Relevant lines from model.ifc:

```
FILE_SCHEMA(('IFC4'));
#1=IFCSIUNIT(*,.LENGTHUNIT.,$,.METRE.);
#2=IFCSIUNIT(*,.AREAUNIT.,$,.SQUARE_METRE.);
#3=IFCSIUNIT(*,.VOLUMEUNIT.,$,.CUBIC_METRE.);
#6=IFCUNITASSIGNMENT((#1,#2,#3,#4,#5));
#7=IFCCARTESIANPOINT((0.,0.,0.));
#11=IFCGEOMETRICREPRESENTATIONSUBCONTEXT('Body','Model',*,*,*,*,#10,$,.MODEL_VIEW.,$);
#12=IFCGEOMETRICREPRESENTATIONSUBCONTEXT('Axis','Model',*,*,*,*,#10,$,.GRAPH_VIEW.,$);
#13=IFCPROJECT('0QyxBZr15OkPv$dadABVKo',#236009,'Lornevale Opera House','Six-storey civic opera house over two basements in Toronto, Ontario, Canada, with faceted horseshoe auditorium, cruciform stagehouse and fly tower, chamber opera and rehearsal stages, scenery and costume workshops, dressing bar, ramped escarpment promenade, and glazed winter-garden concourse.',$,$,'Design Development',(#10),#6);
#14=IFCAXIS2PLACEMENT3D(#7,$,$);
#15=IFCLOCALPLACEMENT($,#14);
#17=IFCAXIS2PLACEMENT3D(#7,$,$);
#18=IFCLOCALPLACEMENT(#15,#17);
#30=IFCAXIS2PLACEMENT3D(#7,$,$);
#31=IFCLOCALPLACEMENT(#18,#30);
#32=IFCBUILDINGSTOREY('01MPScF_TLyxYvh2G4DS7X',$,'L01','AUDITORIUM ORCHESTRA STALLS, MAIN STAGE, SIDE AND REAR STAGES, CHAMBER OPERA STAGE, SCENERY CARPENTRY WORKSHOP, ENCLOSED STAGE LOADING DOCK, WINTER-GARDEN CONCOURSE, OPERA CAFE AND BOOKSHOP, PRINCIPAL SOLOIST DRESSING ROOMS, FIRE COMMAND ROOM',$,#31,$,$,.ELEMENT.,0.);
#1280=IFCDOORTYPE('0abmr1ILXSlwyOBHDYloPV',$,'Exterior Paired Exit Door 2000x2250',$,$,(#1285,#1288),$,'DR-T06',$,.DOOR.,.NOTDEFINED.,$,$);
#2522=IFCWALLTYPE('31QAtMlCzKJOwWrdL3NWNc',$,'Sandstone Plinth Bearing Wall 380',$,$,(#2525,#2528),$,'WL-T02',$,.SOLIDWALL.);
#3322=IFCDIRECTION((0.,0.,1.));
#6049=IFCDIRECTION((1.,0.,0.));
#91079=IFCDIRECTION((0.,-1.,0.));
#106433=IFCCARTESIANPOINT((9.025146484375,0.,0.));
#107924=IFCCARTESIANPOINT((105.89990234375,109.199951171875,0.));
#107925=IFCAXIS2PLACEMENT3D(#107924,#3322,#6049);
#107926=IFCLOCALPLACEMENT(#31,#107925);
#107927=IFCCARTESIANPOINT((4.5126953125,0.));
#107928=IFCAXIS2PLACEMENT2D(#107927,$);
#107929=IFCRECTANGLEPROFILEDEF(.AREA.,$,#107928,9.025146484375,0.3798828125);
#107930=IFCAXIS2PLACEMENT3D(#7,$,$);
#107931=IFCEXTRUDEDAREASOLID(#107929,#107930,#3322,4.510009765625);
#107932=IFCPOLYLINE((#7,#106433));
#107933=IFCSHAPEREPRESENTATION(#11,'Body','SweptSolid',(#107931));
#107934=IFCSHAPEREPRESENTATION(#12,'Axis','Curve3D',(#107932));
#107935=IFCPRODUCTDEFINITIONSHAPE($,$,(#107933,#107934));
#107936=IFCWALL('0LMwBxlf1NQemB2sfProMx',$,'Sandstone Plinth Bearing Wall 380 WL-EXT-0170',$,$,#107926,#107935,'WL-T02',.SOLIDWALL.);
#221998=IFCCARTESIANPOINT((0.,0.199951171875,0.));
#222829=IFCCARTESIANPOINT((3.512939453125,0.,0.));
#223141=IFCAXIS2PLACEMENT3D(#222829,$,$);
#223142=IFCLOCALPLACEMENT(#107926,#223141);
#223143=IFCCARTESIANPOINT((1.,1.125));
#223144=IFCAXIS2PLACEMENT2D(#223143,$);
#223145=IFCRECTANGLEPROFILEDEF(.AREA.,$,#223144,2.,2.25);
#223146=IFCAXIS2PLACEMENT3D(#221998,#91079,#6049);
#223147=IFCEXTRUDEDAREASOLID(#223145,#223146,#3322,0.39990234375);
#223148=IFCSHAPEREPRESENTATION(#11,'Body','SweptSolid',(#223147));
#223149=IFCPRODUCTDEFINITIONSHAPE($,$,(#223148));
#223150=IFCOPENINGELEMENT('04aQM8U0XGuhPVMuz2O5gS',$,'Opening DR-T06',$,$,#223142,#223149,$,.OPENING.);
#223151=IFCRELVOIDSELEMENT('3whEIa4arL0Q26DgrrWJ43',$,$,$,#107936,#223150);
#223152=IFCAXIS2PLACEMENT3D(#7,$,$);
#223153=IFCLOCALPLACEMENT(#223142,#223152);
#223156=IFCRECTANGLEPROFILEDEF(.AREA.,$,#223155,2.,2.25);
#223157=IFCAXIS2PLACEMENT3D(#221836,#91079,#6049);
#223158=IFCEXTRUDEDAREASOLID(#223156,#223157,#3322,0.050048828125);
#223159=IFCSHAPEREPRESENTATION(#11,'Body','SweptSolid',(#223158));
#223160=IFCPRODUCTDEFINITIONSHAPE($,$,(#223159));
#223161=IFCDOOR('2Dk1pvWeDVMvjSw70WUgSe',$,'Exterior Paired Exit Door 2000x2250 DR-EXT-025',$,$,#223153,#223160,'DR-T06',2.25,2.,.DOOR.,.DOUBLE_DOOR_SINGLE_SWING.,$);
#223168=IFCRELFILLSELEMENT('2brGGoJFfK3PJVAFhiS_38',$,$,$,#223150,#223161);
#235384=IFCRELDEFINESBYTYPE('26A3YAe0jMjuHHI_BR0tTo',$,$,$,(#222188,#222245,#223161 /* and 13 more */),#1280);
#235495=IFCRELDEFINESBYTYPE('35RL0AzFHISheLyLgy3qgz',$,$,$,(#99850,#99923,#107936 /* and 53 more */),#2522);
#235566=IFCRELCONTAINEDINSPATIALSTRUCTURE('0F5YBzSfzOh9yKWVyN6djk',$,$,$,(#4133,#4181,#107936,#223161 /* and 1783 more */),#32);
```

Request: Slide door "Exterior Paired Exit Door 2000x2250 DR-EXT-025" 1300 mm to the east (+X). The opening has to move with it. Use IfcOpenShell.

```python
import ifcopenshell
import ifcopenshell.api.geometry
import ifcopenshell.util.placement
import ifcopenshell.util.unit

model = ifcopenshell.open("model.ifc")
unit_scale = ifcopenshell.util.unit.calculate_unit_scale(model)

door = model.by_guid("2Dk1pvWeDVMvjSw70WUgSe")
opening = door.FillsVoids[0].RelatingOpeningElement
wall = opening.VoidsElements[0].RelatingBuildingElement

wall_matrix = ifcopenshell.util.placement.get_local_placement(wall.ObjectPlacement)
shift = wall_matrix[:3, 0] * 1.3 / unit_scale
before = ifcopenshell.util.placement.get_local_placement(door.ObjectPlacement)[:3, 3].copy()

# The door is placed relative to its opening, so it follows when the opening moves.
matrix = ifcopenshell.util.placement.get_local_placement(opening.ObjectPlacement)
matrix[:3, 3] += shift
ifcopenshell.api.geometry.edit_object_placement(
    model, product=opening, matrix=matrix, is_si=False, should_transform_children=True
)

after = ifcopenshell.util.placement.get_local_placement(door.ObjectPlacement)[:3, 3]
print("door moved by", (after - before).round(3) + 0.0)

model.write("model_updated.ifc")
```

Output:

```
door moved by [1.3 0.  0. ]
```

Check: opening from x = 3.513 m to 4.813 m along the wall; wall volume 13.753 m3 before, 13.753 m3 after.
